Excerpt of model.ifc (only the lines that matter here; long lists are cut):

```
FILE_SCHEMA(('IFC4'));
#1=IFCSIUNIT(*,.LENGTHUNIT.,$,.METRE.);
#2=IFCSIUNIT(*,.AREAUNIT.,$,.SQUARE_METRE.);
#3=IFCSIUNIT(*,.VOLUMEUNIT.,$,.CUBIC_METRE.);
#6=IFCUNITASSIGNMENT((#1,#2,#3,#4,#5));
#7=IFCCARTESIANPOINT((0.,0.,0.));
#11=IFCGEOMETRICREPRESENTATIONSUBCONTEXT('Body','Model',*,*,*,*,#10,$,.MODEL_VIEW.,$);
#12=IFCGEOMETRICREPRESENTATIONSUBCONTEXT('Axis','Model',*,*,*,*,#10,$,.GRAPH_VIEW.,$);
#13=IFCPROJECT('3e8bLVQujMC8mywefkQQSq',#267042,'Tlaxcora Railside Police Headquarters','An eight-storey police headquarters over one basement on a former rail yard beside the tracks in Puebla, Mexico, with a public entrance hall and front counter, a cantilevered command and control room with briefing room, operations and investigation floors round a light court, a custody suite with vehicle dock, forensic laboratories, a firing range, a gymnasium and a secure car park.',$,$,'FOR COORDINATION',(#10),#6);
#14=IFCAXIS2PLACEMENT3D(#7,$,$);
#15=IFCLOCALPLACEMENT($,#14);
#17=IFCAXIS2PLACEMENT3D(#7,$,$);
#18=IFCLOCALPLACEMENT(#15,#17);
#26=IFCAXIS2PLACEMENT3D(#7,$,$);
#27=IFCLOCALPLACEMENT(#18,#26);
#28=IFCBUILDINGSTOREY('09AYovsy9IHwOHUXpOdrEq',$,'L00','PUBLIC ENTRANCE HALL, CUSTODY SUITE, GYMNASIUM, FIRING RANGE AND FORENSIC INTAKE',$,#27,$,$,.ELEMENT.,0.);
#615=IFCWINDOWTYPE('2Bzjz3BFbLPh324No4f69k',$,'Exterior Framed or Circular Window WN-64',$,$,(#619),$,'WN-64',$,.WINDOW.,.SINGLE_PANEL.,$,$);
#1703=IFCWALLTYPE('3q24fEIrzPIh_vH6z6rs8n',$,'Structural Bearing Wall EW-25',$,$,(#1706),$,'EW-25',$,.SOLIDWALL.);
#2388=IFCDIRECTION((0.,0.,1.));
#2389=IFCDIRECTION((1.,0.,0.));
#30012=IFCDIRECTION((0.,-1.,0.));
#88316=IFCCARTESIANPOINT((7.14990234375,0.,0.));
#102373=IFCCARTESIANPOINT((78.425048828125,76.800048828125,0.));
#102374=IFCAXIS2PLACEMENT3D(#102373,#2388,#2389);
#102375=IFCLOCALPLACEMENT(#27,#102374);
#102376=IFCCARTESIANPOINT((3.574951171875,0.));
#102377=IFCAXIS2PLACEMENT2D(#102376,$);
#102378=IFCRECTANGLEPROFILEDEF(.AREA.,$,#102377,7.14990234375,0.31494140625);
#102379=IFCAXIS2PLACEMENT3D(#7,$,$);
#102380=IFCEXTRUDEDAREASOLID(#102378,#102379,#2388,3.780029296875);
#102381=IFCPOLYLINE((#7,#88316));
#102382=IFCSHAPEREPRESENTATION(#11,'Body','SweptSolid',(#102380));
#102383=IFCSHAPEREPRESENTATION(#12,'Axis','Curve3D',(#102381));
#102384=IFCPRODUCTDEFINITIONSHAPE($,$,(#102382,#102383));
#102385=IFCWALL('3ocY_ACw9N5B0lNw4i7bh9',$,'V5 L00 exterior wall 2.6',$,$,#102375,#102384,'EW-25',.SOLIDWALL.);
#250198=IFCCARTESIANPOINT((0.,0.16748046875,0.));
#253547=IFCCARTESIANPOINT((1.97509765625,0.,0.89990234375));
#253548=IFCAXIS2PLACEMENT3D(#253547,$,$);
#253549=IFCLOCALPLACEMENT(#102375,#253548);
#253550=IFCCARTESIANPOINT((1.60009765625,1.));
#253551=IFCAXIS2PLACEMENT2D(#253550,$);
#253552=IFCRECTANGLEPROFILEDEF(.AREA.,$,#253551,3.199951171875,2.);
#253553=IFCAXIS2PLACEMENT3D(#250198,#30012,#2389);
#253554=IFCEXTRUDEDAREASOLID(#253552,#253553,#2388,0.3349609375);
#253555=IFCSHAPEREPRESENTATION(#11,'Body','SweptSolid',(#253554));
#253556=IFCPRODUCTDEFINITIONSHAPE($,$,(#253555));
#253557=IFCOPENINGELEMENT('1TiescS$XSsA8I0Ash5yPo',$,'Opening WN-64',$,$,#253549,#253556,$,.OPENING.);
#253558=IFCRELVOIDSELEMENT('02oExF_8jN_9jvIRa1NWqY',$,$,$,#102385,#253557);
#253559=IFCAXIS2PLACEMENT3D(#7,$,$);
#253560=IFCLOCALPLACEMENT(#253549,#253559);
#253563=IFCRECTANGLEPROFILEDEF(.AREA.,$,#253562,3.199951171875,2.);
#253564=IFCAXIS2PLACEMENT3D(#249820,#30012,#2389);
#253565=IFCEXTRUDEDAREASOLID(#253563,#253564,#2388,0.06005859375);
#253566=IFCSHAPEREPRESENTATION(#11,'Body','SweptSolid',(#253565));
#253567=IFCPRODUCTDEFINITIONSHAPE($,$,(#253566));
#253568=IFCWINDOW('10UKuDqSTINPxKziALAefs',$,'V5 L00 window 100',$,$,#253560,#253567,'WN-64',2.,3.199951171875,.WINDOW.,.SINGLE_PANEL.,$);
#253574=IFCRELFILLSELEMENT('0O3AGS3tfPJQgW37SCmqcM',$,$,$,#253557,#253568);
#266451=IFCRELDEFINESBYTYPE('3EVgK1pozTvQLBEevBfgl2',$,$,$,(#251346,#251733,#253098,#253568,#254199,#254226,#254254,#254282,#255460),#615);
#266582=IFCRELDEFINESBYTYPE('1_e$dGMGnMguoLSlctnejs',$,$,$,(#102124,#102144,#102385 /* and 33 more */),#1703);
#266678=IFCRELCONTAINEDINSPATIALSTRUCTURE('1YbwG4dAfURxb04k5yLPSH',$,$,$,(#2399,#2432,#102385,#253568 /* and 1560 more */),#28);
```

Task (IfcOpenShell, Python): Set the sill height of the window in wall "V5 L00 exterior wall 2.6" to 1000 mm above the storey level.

```python
import numpy as np
import ifcopenshell
import ifcopenshell.api.geometry
import ifcopenshell.geom
import ifcopenshell.util.element
import ifcopenshell.util.placement
import ifcopenshell.util.shape
import ifcopenshell.util.unit

model = ifcopenshell.open("model.ifc")
unit_scale = ifcopenshell.util.unit.calculate_unit_scale(model)

window = model.by_id(253568)
opening = window.FillsVoids[0].RelatingOpeningElement
storey = ifcopenshell.util.element.get_container(window, ifc_class="IfcBuildingStorey")
level = ifcopenshell.util.placement.get_local_placement(storey.ObjectPlacement)[2, 3]

# The opening's origin need not be at the sill, so measure its lowest point.
shape = ifcopenshell.geom.create_shape(ifcopenshell.geom.settings(), opening)
bottom = ifcopenshell.util.shape.get_shape_bottom_elevation(shape, shape.geometry) / unit_scale
dz = level + 1 / unit_scale - bottom

shift = np.array([0.0, 0.0, dz])
# The window is placed relative to its opening, so it follows when the opening moves.
matrix = ifcopenshell.util.placement.get_local_placement(opening.ObjectPlacement)
matrix[:3, 3] += shift
ifcopenshell.api.geometry.edit_object_placement(
    model, product=opening, matrix=matrix, is_si=False, should_transform_children=True
)

print(f"moved by {dz * unit_scale:+.3f} m")

model.write("model_updated.ifc")
```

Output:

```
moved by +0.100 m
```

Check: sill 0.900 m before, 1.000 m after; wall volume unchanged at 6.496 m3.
